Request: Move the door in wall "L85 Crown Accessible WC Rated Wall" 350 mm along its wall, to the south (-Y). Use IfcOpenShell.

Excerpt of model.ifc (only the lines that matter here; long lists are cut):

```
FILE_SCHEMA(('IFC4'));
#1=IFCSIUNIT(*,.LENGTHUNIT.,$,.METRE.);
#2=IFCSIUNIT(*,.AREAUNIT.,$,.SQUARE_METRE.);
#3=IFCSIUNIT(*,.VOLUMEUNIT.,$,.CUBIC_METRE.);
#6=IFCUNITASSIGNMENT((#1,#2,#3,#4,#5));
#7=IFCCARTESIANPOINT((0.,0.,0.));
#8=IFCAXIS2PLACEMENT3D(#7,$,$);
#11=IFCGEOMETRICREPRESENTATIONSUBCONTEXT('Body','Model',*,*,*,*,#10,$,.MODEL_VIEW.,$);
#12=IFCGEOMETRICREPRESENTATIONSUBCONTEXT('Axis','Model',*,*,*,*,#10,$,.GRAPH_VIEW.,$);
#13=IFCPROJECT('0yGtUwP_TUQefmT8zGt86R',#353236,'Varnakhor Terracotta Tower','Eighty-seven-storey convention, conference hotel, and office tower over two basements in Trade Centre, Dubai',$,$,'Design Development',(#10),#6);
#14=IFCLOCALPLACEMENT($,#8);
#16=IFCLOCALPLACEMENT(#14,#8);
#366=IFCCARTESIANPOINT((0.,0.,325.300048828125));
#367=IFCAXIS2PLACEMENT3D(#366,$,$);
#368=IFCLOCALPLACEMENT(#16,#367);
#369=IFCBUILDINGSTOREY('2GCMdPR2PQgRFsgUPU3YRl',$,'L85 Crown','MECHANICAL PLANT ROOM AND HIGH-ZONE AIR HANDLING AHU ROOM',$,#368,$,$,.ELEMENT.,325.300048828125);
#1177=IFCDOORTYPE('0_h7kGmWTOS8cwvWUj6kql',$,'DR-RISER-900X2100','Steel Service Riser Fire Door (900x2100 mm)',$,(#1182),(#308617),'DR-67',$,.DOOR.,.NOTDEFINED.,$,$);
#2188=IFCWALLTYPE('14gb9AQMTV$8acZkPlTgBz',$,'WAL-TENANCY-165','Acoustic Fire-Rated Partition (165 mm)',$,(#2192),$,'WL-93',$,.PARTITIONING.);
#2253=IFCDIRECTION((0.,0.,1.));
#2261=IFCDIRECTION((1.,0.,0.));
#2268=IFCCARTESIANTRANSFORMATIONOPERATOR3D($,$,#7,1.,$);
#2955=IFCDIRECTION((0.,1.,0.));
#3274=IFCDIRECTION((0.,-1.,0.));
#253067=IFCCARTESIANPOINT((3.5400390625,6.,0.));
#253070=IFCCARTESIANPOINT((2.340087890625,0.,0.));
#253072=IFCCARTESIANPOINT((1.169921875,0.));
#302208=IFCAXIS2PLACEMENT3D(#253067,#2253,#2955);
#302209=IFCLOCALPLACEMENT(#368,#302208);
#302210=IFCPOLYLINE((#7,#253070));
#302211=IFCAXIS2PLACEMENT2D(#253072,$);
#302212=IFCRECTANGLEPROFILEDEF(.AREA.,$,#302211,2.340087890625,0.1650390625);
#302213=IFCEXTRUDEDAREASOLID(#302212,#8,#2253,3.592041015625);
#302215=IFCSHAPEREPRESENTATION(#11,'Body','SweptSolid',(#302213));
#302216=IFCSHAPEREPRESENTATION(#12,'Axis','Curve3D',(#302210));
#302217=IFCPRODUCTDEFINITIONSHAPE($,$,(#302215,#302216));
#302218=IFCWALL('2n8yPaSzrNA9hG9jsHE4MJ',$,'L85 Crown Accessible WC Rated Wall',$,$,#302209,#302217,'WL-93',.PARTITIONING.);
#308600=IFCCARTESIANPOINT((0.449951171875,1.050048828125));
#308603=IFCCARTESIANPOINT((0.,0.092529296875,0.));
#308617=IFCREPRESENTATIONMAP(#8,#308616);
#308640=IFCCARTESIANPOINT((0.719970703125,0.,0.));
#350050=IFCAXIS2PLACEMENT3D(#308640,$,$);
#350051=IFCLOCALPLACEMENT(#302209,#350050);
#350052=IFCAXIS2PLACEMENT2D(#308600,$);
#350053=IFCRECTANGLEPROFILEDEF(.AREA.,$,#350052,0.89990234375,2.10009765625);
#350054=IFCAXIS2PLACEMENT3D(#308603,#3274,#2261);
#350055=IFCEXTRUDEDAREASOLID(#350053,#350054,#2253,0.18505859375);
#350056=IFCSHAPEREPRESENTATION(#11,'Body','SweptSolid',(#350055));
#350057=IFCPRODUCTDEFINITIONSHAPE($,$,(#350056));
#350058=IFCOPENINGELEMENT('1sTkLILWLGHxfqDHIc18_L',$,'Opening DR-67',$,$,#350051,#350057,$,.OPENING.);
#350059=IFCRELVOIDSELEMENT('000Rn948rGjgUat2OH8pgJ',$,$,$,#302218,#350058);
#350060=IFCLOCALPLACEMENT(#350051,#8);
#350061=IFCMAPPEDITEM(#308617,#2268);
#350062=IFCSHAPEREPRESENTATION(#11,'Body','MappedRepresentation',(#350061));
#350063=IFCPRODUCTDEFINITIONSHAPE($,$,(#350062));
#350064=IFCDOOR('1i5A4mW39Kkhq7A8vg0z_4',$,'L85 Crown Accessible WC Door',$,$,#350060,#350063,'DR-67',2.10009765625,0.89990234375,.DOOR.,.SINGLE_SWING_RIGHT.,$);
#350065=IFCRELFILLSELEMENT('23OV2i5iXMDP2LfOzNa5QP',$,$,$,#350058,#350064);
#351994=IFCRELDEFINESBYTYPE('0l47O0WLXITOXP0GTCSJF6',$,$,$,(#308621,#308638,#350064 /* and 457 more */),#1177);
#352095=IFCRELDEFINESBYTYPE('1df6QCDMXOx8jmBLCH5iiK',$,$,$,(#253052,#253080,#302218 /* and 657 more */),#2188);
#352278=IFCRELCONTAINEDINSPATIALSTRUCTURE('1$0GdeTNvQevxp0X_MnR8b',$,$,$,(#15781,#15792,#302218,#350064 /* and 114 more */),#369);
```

```python
import ifcopenshell
import ifcopenshell.api.geometry
import ifcopenshell.util.placement
import ifcopenshell.util.unit

model = ifcopenshell.open("model.ifc")
unit_scale = ifcopenshell.util.unit.calculate_unit_scale(model)

door = model.by_guid("1i5A4mW39Kkhq7A8vg0z_4")
opening = door.FillsVoids[0].RelatingOpeningElement
wall = opening.VoidsElements[0].RelatingBuildingElement

wall_matrix = ifcopenshell.util.placement.get_local_placement(wall.ObjectPlacement)
shift = wall_matrix[:3, 0] * -0.35 / unit_scale
before = ifcopenshell.util.placement.get_local_placement(door.ObjectPlacement)[:3, 3].copy()

# The door is placed relative to its opening, so it follows when the opening moves.
matrix = ifcopenshell.util.placement.get_local_placement(opening.ObjectPlacement)
matrix[:3, 3] += shift
ifcopenshell.api.geometry.edit_object_placement(
    model, product=opening, matrix=matrix, is_si=False, should_transform_children=True
)

after = ifcopenshell.util.placement.get_local_placement(door.ObjectPlacement)[:3, 3]
print("door moved by", (after - before).round(3) + 0.0)

model.write("model-out.ifc")
```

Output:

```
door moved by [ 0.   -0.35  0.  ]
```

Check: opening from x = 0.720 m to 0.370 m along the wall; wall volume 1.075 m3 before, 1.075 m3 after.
